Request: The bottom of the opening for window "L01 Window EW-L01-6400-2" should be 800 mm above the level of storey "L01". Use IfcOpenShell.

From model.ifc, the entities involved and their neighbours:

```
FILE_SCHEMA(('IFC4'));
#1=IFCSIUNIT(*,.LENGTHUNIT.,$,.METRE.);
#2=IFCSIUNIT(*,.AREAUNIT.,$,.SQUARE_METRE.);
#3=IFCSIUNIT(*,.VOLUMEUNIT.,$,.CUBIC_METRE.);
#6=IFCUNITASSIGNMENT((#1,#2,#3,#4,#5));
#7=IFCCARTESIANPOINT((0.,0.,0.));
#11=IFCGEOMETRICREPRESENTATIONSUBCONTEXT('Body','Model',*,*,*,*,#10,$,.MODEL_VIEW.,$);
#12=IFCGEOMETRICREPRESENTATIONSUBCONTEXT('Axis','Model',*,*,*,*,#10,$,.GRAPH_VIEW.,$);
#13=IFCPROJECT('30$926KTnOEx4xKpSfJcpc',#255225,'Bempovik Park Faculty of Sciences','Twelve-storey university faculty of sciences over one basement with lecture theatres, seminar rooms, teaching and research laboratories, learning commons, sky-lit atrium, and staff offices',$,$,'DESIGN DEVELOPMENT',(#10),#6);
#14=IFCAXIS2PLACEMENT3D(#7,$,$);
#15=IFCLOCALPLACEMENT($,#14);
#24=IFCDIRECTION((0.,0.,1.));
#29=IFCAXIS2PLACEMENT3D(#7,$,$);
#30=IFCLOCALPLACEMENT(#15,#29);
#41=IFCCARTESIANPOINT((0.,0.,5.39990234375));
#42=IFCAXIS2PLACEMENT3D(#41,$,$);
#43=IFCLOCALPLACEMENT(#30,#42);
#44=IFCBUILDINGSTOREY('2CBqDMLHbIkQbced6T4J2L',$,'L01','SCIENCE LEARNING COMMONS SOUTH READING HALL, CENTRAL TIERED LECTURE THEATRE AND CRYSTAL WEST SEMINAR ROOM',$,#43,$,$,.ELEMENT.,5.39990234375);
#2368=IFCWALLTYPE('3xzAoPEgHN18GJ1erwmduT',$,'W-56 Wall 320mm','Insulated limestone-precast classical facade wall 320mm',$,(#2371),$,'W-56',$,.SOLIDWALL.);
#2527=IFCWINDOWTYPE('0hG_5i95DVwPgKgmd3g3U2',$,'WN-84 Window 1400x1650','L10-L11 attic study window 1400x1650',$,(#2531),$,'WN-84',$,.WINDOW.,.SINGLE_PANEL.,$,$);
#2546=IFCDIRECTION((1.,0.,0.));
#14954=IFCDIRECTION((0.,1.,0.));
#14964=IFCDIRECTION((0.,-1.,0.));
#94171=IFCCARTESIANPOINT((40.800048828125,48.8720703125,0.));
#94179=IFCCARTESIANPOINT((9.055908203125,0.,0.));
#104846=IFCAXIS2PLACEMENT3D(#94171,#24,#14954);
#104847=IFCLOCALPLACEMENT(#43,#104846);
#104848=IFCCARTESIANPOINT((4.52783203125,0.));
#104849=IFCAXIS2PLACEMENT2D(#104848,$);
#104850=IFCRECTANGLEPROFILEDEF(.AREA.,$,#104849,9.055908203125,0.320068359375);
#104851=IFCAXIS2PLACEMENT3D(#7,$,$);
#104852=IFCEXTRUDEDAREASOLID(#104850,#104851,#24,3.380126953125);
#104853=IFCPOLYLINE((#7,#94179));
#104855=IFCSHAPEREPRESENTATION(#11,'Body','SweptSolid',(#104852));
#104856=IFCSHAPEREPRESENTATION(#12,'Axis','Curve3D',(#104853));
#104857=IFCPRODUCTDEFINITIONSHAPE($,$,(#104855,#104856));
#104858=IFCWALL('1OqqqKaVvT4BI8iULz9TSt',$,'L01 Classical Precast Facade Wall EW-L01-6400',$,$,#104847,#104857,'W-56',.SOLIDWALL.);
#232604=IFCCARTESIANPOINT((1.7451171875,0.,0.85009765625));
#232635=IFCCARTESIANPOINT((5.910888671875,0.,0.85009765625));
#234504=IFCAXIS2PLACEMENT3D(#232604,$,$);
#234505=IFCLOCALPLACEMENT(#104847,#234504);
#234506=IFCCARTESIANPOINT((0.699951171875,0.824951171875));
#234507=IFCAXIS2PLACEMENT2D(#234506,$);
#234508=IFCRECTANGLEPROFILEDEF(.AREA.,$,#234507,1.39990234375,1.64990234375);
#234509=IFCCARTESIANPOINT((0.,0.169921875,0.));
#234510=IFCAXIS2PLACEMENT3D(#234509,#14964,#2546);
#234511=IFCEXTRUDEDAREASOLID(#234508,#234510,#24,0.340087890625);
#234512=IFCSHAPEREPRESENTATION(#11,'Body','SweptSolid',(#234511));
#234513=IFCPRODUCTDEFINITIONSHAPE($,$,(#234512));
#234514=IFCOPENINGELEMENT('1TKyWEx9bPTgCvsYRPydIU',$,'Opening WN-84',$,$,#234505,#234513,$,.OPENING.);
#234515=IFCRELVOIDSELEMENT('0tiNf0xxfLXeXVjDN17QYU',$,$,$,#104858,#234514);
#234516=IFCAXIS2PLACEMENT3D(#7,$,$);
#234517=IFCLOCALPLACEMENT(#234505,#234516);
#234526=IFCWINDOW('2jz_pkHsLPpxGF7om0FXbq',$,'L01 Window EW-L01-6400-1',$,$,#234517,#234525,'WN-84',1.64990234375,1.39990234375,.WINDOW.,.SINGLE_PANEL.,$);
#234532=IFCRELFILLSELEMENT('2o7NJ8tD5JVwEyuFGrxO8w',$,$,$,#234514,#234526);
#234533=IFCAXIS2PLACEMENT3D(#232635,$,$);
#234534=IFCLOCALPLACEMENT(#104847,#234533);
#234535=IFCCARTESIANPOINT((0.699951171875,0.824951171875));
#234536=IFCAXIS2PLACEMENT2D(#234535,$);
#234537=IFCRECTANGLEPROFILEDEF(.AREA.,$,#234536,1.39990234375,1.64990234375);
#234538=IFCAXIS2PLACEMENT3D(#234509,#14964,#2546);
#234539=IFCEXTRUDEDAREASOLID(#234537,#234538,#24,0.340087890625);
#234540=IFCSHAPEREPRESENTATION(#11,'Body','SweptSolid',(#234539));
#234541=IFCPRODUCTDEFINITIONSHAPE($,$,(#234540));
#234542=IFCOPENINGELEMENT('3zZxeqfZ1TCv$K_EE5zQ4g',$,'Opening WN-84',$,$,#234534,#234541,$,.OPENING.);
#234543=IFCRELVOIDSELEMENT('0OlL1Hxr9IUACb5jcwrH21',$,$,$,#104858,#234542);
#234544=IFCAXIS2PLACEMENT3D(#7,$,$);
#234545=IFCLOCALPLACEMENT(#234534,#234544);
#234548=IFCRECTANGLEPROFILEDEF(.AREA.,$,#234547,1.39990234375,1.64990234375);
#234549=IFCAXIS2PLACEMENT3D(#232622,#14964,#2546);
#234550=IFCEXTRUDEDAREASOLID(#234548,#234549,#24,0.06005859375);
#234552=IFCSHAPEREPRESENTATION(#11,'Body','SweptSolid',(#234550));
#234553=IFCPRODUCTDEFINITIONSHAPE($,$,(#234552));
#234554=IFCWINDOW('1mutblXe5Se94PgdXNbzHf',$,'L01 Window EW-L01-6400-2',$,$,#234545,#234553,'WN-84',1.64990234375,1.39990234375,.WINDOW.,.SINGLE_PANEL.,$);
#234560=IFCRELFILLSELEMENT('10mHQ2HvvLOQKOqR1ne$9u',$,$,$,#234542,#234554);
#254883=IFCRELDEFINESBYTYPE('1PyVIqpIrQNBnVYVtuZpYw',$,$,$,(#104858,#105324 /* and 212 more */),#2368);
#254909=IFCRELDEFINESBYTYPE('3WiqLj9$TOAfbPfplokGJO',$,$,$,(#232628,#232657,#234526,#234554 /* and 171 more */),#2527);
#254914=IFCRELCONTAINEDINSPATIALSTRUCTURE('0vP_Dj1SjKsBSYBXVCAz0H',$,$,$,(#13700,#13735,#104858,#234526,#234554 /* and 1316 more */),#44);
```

```python
import numpy as np
import ifcopenshell
import ifcopenshell.api.geometry
import ifcopenshell.geom
import ifcopenshell.util.element
import ifcopenshell.util.placement
import ifcopenshell.util.shape
import ifcopenshell.util.unit

model = ifcopenshell.open("model.ifc")
unit_scale = ifcopenshell.util.unit.calculate_unit_scale(model)

window = model.by_id(234554)
opening = window.FillsVoids[0].RelatingOpeningElement
storey = ifcopenshell.util.element.get_container(window, ifc_class="IfcBuildingStorey")
level = ifcopenshell.util.placement.get_local_placement(storey.ObjectPlacement)[2, 3]

# The opening's origin need not be at the sill, so measure its lowest point.
shape = ifcopenshell.geom.create_shape(ifcopenshell.geom.settings(), opening)
bottom = ifcopenshell.util.shape.get_shape_bottom_elevation(shape, shape.geometry) / unit_scale
dz = level + 0.8 / unit_scale - bottom

shift = np.array([0.0, 0.0, dz])
# The window is placed relative to its opening, so it follows when the opening moves.
matrix = ifcopenshell.util.placement.get_local_placement(opening.ObjectPlacement)
matrix[:3, 3] += shift
ifcopenshell.api.geometry.edit_object_placement(
    model, product=opening, matrix=matrix, is_si=False, should_transform_children=True
)

print(f"moved by {dz * unit_scale:+.3f} m")

model.write("model_rev.ifc")
```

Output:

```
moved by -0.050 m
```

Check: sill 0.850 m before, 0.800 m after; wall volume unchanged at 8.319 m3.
